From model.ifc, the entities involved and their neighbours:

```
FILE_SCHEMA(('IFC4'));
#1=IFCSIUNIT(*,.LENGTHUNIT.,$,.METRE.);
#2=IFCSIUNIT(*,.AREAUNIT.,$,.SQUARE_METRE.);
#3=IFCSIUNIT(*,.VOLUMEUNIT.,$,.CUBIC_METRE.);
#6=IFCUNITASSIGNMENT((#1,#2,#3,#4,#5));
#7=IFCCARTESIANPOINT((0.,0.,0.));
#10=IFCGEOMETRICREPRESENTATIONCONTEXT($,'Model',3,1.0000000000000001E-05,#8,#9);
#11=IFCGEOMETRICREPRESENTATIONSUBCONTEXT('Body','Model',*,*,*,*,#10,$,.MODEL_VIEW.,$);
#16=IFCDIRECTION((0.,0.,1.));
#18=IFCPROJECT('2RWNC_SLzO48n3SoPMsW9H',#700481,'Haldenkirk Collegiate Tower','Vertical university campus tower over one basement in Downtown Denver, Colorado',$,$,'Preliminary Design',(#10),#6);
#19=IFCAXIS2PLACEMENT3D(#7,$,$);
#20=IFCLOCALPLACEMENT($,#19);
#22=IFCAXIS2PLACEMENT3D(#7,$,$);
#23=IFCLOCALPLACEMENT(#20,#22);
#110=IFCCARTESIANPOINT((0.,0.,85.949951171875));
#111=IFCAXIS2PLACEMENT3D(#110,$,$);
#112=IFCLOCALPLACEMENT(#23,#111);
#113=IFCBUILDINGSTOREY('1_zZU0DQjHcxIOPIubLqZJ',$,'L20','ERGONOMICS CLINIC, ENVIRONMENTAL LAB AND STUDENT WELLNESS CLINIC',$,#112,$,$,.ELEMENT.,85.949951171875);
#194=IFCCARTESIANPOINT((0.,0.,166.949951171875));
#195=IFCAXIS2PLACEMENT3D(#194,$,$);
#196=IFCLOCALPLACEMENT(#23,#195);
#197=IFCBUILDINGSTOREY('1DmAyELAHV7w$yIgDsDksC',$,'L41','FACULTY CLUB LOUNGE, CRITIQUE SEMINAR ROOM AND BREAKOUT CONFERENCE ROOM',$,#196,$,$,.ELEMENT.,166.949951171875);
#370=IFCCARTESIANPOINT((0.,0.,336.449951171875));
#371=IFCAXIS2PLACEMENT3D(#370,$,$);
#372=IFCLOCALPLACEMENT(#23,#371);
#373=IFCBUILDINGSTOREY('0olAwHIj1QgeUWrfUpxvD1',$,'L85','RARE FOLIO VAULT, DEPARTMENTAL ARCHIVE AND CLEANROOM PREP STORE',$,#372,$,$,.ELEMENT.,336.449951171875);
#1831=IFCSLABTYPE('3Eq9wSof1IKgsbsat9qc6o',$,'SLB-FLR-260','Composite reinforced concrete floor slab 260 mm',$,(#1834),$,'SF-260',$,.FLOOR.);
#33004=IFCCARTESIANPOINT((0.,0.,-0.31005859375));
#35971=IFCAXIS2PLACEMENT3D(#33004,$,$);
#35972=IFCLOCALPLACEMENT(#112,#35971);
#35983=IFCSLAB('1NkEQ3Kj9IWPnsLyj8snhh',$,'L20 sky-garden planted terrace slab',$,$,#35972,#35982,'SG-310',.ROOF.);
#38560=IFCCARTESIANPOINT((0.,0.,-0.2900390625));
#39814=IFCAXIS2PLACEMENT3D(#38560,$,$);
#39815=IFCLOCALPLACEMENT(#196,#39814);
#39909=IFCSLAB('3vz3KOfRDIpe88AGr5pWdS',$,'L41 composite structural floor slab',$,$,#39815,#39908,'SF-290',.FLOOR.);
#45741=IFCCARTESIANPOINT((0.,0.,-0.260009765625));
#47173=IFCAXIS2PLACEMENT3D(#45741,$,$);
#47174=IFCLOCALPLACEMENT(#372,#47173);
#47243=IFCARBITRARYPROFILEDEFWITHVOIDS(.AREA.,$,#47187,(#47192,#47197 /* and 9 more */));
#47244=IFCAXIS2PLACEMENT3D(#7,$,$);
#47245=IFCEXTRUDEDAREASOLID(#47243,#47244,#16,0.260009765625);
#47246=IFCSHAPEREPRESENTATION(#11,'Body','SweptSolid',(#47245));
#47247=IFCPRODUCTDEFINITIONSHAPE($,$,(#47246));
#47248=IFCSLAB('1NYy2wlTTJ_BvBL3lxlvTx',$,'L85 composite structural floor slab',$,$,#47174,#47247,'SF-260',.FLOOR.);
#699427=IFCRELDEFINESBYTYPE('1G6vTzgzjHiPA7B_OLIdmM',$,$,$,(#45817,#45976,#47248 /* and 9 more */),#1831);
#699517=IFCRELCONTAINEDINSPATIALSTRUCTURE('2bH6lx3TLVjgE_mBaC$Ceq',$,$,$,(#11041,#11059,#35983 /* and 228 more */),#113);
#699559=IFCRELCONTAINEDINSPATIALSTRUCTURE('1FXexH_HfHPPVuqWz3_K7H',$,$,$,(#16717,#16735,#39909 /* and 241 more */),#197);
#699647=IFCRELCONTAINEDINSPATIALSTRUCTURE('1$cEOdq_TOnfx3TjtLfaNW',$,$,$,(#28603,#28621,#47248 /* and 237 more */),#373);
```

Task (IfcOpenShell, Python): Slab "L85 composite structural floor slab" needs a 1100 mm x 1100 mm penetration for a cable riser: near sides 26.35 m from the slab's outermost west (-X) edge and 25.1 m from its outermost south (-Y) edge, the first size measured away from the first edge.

```python
import numpy as np
import ifcopenshell
import ifcopenshell.api.feature
import ifcopenshell.api.geometry
import ifcopenshell.api.root
import ifcopenshell.geom
import ifcopenshell.util.placement
import ifcopenshell.util.representation
import ifcopenshell.util.shape
import ifcopenshell.util.unit

model = ifcopenshell.open("model.ifc")
unit_scale = ifcopenshell.util.unit.calculate_unit_scale(model)
settings = ifcopenshell.geom.settings()


def volume(element):
    """Net volume in cubic metres, openings subtracted."""
    shape = ifcopenshell.geom.create_shape(settings, element)
    return ifcopenshell.util.shape.get_volume(shape.geometry)


slab = model.by_id(47248)
before = volume(slab)

# Extent in the slab's own axes, in metres. The edges named are its -X and -Y sides.
slab_shape = ifcopenshell.geom.create_shape(settings, slab)
vertices = ifcopenshell.util.shape.get_vertices(slab_shape.geometry)
x_min, y_min, bottom = vertices.min(axis=0)
top = vertices[:, 2].max()

opening = ifcopenshell.api.root.create_entity(model, ifc_class="IfcOpeningElement", name="Cable riser opening", predefined_type="OPENING")
context = ifcopenshell.util.representation.get_context(model, "Model", "Body", "MODEL_VIEW")
width, depth = 1.1, 1.1
outline = [(0.0, 0.0), (width, 0.0), (width, depth), (0.0, depth), (0.0, 0.0)]
# Overshoot both faces by 50 mm so the cut is clean.
shape = ifcopenshell.api.geometry.add_slab_representation(
    model, context=context, depth=top - bottom + 0.1, polyline=outline
)
ifcopenshell.api.geometry.assign_representation(model, product=opening, representation=shape)

matrix = ifcopenshell.util.placement.get_local_placement(slab.ObjectPlacement)
matrix[:, 3] = matrix @ np.append(np.array([x_min + 26.35, y_min + 25.1, bottom - 0.05]) / unit_scale, 1.0)
ifcopenshell.api.geometry.edit_object_placement(model, product=opening, matrix=matrix, is_si=False)
ifcopenshell.api.feature.add_feature(model, feature=opening, element=slab)

after = volume(slab)

print(f"slab volume {before:.3f} -> {after:.3f} m3")

model.write("model-out.ifc")
```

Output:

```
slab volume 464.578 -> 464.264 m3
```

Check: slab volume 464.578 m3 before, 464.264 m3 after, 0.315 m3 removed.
